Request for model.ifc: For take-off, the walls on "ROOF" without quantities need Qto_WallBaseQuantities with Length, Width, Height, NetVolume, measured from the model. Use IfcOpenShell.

First a look at what the model holds.

```python
import ifcopenshell
import ifcopenshell.util.element
import ifcopenshell.util.unit

model = ifcopenshell.open("model.ifc")
print(model.schema)
for unit_type in ("LENGTHUNIT", "AREAUNIT", "VOLUMEUNIT"):
    print(unit_type, ifcopenshell.util.unit.calculate_unit_scale(model, unit_type))
storey = next(s for s in model.by_type("IfcBuildingStorey") if s.Name == "ROOF")
walls = [e for e in ifcopenshell.util.element.get_decomposition(storey) if e.is_a("IfcWall")]
for e in sorted(walls, key=lambda e: e.id()):
    print(e.id(), e.is_a(), e.Name, list(ifcopenshell.util.element.get_psets(e, qtos_only=True)), sep=" | ")
```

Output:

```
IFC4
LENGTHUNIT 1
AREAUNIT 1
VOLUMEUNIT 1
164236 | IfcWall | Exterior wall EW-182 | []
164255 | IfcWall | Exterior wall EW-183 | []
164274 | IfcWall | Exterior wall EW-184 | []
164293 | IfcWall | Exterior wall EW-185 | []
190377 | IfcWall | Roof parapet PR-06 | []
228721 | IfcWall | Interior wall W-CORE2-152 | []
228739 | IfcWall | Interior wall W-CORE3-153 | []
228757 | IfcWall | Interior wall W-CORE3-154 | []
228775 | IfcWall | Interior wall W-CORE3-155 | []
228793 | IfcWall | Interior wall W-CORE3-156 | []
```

```python
import ifcopenshell
import ifcopenshell.api.pset
import ifcopenshell.geom
import ifcopenshell.util.element
import ifcopenshell.util.shape
import ifcopenshell.util.unit

model = ifcopenshell.open("model.ifc")
unit_scale = ifcopenshell.util.unit.calculate_unit_scale(model)
volume_scale = ifcopenshell.util.unit.calculate_unit_scale(model, "VOLUMEUNIT")
settings = ifcopenshell.geom.settings()

storey = next(s for s in model.by_type("IfcBuildingStorey") if s.Name == "ROOF")
walls = [e for e in ifcopenshell.util.element.get_decomposition(storey) if e.is_a("IfcWall")]

for e in sorted(walls, key=lambda e: e.id()):
    if ifcopenshell.util.element.get_psets(e, qtos_only=True, should_inherit=False):
        continue
    # Geometry comes back in metres, in the element's own axes.
    shape = ifcopenshell.geom.create_shape(settings, e)
    values = {
        "Length": ifcopenshell.util.shape.get_x(shape.geometry) / unit_scale,
        "Width": ifcopenshell.util.shape.get_y(shape.geometry) / unit_scale,
        "Height": ifcopenshell.util.shape.get_z(shape.geometry) / unit_scale,
        "NetVolume": ifcopenshell.util.shape.get_volume(shape.geometry) / volume_scale,
    }
    qto = ifcopenshell.api.pset.add_qto(model, product=e, name="Qto_WallBaseQuantities")
    ifcopenshell.api.pset.edit_qto(model, qto=qto, properties=values)
    print(e.id(), {k: round(v, 3) for k, v in values.items()})

model.write("model-out.ifc")
```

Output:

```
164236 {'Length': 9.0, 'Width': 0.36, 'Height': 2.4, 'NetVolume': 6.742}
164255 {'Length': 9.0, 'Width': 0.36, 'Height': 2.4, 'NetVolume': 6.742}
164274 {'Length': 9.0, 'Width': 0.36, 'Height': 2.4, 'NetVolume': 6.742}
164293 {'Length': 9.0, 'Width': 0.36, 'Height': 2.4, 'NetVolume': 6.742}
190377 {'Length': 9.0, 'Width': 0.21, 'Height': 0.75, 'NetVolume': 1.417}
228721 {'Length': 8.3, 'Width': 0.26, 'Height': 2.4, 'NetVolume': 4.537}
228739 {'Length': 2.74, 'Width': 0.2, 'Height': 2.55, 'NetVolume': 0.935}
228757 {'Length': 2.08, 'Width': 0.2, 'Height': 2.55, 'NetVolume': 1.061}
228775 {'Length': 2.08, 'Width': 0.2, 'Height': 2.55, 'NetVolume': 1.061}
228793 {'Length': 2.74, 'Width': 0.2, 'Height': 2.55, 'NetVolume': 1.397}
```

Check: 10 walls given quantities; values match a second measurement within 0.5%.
